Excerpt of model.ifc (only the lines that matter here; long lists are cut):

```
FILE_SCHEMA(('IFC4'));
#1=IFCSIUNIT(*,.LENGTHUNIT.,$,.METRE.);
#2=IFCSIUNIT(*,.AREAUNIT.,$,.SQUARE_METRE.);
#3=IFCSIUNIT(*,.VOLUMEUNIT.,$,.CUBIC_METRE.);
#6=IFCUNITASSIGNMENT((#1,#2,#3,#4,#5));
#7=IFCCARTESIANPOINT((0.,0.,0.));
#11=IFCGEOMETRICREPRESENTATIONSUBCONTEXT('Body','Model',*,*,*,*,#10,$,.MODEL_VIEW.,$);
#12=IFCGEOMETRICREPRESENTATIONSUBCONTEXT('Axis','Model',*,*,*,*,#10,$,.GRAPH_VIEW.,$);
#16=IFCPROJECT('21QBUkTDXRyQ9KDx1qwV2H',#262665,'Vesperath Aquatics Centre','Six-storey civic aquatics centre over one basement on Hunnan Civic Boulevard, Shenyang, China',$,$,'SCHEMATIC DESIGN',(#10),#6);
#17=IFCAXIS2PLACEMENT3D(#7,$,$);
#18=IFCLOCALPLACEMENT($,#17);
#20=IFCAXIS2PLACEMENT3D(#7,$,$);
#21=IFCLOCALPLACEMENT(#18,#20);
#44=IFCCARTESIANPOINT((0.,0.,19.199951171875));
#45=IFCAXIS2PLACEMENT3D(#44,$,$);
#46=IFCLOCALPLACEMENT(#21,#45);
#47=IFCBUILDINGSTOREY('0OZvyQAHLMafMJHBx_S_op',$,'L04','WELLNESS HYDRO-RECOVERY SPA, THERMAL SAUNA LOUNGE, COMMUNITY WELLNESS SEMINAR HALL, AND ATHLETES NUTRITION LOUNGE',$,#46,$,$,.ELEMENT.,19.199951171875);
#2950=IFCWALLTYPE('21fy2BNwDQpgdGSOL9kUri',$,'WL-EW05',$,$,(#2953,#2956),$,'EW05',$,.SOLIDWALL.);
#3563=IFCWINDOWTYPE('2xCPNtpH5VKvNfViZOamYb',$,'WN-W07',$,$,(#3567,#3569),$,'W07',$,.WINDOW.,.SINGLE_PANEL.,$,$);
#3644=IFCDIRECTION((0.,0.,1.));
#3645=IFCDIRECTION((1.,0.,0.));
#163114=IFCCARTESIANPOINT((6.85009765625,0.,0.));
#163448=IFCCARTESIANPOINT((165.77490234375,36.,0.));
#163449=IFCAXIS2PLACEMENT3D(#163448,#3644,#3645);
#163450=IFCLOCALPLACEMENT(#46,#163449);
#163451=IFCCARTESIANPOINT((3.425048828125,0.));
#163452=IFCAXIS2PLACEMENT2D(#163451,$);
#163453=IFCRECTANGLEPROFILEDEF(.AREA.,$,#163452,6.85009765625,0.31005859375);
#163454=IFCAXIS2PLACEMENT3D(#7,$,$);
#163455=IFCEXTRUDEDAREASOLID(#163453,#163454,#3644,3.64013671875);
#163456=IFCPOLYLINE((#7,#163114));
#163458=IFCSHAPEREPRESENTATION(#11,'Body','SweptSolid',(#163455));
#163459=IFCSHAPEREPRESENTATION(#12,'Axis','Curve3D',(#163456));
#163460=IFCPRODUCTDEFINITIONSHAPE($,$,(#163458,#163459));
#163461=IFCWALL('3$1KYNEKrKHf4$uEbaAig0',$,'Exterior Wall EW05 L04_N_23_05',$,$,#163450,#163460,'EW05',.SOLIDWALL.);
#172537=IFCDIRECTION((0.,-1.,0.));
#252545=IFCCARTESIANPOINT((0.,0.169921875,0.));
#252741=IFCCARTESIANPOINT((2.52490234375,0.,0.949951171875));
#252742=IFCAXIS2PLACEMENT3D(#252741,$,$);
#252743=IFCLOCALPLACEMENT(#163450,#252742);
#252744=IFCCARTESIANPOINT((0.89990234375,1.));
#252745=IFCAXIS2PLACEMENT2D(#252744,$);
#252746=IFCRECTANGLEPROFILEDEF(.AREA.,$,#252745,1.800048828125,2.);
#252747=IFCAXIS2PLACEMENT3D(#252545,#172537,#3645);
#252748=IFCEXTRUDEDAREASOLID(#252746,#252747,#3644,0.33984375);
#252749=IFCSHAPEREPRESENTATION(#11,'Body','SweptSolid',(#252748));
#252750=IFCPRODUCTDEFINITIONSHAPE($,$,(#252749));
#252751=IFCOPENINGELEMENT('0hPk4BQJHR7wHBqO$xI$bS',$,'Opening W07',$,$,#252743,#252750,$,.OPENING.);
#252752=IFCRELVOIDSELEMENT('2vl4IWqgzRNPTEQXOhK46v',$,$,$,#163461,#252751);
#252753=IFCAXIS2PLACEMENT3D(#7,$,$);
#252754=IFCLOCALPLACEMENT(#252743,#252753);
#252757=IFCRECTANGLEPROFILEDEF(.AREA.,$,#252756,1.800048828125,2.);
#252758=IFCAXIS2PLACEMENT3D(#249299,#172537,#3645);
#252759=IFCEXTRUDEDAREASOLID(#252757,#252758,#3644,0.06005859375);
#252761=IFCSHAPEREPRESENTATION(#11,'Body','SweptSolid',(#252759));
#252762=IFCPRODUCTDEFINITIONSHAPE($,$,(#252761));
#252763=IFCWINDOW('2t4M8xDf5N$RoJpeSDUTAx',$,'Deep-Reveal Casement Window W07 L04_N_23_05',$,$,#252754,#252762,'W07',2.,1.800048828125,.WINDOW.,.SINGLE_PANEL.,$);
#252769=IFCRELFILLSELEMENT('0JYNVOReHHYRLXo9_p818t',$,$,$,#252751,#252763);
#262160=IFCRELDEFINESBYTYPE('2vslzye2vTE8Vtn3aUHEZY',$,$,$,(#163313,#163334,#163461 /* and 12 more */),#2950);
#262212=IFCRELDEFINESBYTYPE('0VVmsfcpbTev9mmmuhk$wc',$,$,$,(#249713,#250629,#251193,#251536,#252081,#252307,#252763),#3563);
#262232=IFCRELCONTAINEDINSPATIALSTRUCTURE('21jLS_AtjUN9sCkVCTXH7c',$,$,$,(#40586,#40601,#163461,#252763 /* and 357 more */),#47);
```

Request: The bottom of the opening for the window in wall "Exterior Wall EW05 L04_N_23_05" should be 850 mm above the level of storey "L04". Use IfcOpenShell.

```python
import numpy as np
import ifcopenshell
import ifcopenshell.api.geometry
import ifcopenshell.geom
import ifcopenshell.util.element
import ifcopenshell.util.placement
import ifcopenshell.util.shape
import ifcopenshell.util.unit

model = ifcopenshell.open("model.ifc")
unit_scale = ifcopenshell.util.unit.calculate_unit_scale(model)

window = model.by_guid("2t4M8xDf5N$RoJpeSDUTAx")
opening = window.FillsVoids[0].RelatingOpeningElement
storey = ifcopenshell.util.element.get_container(window, ifc_class="IfcBuildingStorey")
level = ifcopenshell.util.placement.get_local_placement(storey.ObjectPlacement)[2, 3]

# The opening's origin need not be at the sill, so measure its lowest point.
shape = ifcopenshell.geom.create_shape(ifcopenshell.geom.settings(), opening)
bottom = ifcopenshell.util.shape.get_shape_bottom_elevation(shape, shape.geometry) / unit_scale
dz = level + 0.85 - bottom

shift = np.array([0.0, 0.0, dz])
# The window is placed relative to its opening, so it follows when the opening moves.
matrix = ifcopenshell.util.placement.get_local_placement(opening.ObjectPlacement)
matrix[:3, 3] += shift
ifcopenshell.api.geometry.edit_object_placement(
    model, product=opening, matrix=matrix, is_si=False, should_transform_children=True
)

print(f"moved by {dz * unit_scale:+.3f} m")

model.write("model_updated.ifc")
```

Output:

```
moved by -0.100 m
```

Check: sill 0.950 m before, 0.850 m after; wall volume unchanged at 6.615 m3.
